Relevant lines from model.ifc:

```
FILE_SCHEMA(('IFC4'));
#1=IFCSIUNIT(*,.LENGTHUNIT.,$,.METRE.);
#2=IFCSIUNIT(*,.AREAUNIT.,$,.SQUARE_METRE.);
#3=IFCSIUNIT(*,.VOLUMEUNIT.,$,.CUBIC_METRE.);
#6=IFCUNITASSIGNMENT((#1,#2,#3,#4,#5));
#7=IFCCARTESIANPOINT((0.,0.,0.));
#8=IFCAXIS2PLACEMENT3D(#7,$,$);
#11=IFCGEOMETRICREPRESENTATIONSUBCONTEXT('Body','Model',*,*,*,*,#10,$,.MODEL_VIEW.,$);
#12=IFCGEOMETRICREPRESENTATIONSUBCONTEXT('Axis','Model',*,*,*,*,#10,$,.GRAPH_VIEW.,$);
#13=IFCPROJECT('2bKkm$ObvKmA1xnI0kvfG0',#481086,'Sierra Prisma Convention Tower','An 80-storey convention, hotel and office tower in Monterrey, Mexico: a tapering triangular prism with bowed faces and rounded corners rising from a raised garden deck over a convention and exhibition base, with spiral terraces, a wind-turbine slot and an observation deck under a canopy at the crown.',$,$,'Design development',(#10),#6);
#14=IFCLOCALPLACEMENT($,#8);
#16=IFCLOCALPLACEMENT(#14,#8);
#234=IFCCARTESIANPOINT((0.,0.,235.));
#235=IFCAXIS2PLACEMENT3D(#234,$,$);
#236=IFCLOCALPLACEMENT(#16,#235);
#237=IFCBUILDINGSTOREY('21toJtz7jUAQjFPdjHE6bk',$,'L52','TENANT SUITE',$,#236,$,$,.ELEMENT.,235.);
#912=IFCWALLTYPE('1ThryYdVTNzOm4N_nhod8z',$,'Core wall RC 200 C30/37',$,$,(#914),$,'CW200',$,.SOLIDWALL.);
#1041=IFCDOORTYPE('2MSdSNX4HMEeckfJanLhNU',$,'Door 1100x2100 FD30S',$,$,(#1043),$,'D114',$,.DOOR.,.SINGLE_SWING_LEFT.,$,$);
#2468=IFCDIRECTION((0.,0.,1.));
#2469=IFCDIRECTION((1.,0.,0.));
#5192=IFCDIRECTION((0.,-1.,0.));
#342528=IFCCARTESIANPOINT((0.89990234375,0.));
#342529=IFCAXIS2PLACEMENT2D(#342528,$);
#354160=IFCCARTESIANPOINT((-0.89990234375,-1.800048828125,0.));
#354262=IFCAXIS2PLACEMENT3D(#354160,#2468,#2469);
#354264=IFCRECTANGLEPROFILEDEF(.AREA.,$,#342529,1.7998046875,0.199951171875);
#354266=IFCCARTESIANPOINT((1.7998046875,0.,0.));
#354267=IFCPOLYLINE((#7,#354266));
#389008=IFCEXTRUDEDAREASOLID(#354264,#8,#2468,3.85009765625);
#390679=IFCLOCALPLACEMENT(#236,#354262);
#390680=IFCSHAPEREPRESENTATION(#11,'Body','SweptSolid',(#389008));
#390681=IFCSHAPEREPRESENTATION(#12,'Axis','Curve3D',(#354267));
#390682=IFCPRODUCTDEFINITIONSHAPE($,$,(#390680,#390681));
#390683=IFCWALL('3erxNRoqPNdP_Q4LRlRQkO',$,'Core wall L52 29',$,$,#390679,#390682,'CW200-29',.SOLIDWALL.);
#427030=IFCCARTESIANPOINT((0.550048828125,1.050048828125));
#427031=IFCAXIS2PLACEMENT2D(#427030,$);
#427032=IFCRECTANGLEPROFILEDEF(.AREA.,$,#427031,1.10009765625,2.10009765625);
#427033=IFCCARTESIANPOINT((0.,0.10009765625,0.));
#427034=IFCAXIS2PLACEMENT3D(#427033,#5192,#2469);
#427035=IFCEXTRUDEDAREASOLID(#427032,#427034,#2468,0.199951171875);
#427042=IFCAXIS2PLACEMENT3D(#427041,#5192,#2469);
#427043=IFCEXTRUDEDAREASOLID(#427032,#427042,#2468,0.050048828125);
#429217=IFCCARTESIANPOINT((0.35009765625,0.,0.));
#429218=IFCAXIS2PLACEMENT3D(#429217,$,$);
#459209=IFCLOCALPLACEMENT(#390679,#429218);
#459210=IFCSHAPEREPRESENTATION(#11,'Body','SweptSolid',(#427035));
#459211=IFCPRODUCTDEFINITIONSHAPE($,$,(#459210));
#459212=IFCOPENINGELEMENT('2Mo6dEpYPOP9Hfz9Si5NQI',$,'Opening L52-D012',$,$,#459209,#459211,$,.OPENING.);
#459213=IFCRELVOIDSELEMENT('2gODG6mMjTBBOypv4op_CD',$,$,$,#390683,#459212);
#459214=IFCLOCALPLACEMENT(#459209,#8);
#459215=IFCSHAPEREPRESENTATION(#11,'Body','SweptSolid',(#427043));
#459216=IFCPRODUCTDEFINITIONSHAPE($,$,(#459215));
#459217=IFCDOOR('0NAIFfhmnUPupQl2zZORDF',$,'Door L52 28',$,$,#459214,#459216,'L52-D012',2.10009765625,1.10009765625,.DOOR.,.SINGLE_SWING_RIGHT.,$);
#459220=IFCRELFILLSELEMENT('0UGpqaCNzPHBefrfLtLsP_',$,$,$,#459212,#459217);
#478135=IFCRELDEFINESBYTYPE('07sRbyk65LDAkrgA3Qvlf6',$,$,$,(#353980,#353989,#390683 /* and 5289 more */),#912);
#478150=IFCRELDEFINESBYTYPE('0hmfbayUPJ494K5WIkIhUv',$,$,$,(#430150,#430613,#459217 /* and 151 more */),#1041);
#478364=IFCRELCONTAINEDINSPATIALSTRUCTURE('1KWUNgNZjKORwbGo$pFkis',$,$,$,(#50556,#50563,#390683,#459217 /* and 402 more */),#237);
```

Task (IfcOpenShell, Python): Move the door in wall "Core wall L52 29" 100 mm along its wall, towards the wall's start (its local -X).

```python
import ifcopenshell
import ifcopenshell.api.geometry
import ifcopenshell.util.placement

model = ifcopenshell.open("model.ifc")

door = model.by_guid("0NAIFfhmnUPupQl2zZORDF")
opening = door.FillsVoids[0].RelatingOpeningElement
wall = opening.VoidsElements[0].RelatingBuildingElement

wall_matrix = ifcopenshell.util.placement.get_local_placement(wall.ObjectPlacement)
shift = wall_matrix[:3, 0] * -0.1
before = ifcopenshell.util.placement.get_local_placement(door.ObjectPlacement)[:3, 3].copy()

# The door is placed relative to its opening, so it follows when the opening moves.
matrix = ifcopenshell.util.placement.get_local_placement(opening.ObjectPlacement)
matrix[:3, 3] += shift
ifcopenshell.api.geometry.edit_object_placement(
    model, product=opening, matrix=matrix, is_si=False, should_transform_children=True
)

after = ifcopenshell.util.placement.get_local_placement(door.ObjectPlacement)[:3, 3]
print("door moved by", (after - before).round(3) + 0.0)

model.write("model_rev.ifc")
```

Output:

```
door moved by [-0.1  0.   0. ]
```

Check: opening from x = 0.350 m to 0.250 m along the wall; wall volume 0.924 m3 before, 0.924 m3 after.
